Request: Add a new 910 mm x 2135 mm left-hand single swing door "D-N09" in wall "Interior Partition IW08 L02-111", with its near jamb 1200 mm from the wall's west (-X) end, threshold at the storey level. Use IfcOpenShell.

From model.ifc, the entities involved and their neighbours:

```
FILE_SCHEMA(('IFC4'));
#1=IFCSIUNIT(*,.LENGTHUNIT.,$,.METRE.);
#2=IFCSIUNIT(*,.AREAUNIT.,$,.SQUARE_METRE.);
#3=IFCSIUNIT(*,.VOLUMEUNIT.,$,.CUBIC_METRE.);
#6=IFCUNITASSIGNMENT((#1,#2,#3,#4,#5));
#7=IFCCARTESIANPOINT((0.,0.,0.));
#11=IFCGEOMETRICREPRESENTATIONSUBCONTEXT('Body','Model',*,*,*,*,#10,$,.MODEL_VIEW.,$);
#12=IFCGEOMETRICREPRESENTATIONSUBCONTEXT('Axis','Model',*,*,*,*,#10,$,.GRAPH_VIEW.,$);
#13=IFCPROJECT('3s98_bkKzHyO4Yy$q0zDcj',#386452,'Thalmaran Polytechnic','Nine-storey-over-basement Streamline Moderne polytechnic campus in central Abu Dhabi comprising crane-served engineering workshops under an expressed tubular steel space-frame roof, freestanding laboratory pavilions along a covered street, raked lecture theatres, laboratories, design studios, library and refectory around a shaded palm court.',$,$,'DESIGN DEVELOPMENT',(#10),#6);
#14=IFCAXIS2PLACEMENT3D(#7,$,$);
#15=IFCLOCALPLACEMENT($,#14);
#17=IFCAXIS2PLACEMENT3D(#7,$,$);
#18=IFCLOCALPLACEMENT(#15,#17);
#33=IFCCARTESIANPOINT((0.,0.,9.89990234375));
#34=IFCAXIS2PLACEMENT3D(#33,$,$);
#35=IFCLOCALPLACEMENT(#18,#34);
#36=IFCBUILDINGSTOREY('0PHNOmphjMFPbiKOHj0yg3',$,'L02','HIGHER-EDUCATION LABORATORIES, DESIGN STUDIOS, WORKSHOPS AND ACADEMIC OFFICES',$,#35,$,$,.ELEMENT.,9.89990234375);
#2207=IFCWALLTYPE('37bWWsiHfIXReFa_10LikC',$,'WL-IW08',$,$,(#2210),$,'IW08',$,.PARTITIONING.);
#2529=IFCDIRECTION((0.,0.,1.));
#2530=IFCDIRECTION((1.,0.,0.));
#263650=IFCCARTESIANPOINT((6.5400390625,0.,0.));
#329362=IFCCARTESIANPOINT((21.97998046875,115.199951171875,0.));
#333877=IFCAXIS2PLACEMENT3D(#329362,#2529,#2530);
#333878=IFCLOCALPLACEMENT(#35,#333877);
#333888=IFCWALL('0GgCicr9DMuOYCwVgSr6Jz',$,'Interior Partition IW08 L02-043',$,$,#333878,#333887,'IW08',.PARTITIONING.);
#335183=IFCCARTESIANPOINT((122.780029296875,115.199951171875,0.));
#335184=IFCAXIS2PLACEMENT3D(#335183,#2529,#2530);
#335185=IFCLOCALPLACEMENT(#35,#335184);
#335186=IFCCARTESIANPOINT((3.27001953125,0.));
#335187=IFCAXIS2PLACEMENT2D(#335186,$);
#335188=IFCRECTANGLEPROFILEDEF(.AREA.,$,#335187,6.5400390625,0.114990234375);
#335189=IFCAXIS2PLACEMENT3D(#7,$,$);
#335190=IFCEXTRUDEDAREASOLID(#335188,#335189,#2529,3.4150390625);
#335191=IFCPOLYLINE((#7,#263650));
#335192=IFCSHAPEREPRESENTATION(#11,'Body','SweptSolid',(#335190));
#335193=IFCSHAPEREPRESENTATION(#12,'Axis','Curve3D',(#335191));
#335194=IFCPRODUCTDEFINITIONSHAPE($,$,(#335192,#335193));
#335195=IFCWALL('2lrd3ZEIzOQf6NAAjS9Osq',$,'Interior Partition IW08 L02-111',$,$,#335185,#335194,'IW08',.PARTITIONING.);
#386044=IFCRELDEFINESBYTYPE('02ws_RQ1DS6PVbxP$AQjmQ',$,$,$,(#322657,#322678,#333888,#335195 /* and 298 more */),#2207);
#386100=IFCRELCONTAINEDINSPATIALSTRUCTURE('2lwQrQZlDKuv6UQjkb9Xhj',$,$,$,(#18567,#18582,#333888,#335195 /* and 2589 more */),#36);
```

```python
import numpy as np
import ifcopenshell
import ifcopenshell.api.feature
import ifcopenshell.api.geometry
import ifcopenshell.api.root
import ifcopenshell.api.spatial
import ifcopenshell.geom
import ifcopenshell.util.element
import ifcopenshell.util.placement
import ifcopenshell.util.representation
import ifcopenshell.util.shape
import ifcopenshell.util.unit

model = ifcopenshell.open("model.ifc")
unit_scale = ifcopenshell.util.unit.calculate_unit_scale(model)
settings = ifcopenshell.geom.settings()


def volume(element):
    """Net volume in cubic metres, openings subtracted."""
    shape = ifcopenshell.geom.create_shape(settings, element)
    return ifcopenshell.util.shape.get_volume(shape.geometry)


wall = model.by_guid("2lrd3ZEIzOQf6NAAjS9Osq")
storey = ifcopenshell.util.element.get_container(wall, ifc_class="IfcBuildingStorey")
context = ifcopenshell.util.representation.get_context(model, "Model", "Body", "MODEL_VIEW")
before = volume(wall)

width, height, from_end, sill = 0.91, 2.135, 1.2, 0.0  # metres

# The wall runs along its own X axis, and the end named is its -X end.
wall_shape = ifcopenshell.geom.create_shape(settings, wall)
x, y, z = ifcopenshell.util.shape.get_vertices(wall_shape.geometry).T
start = x.min() + from_end
face, thickness = float(y.min()), float(y.max() - y.min())
wall_matrix = ifcopenshell.util.placement.get_local_placement(wall.ObjectPlacement)
level = ifcopenshell.util.placement.get_local_placement(storey.ObjectPlacement)[2, 3]


def in_wall(x, y):
    """Placement at x, y metres in the wall's axes, at sill height."""
    matrix = wall_matrix.copy()
    matrix[:, 3] = wall_matrix @ np.array([x / unit_scale, y / unit_scale, 0.0, 1.0])
    matrix[2, 3] = level + sill / unit_scale
    return matrix


# Opening: a box that overshoots both wall faces by 50 mm.
opening = ifcopenshell.api.root.create_entity(model, ifc_class="IfcOpeningElement", predefined_type="OPENING")
box = ifcopenshell.api.geometry.add_wall_representation(
    model, context=context, length=width, height=height, thickness=thickness + 0.1
)
ifcopenshell.api.geometry.assign_representation(model, product=opening, representation=box)
ifcopenshell.api.geometry.edit_object_placement(model, product=opening, matrix=in_wall(start, face - 0.05), is_si=False)
ifcopenshell.api.feature.add_feature(model, feature=opening, element=wall)

door = ifcopenshell.api.root.create_entity(model, ifc_class="IfcDoor", name="D-N09", predefined_type="DOOR")
door.OverallWidth, door.OverallHeight = width / unit_scale, height / unit_scale
door.OperationType = "SINGLE_SWING_LEFT"
body = ifcopenshell.api.geometry.add_door_representation(
    model,
    context=context,
    overall_width=door.OverallWidth,
    overall_height=door.OverallHeight,
    operation_type="SINGLE_SWING_LEFT",
    lining_properties={"LiningDepth": thickness / unit_scale, "ThresholdDepth": thickness / unit_scale},
)
ifcopenshell.api.geometry.assign_representation(model, product=door, representation=body)
ifcopenshell.api.spatial.assign_container(model, products=[door], relating_structure=storey)
ifcopenshell.api.feature.add_filling(model, opening=opening, element=door)

# The lining spans the wall, so the door starts at the wall face.
ifcopenshell.api.geometry.edit_object_placement(model, product=door, matrix=in_wall(start, face), is_si=False)

after = volume(wall)

print(f"wall volume {before:.3f} -> {after:.3f} m3")

model.write("model_v2.ifc")
```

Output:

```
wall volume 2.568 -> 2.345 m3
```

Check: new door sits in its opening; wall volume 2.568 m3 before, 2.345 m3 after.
